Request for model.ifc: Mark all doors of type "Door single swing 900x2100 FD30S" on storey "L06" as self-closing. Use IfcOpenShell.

First a look at what the model holds.

```python
import ifcopenshell
import ifcopenshell.util.element

model = ifcopenshell.open("model.ifc")
print(model.schema)
storey = next(s for s in model.by_type("IfcBuildingStorey") if s.Name == "L06")
doors = [e for e in ifcopenshell.util.element.get_decomposition(storey) if e.is_a("IfcDoor")]
seen = {}
for e in doors:
    element_type = ifcopenshell.util.element.get_type(e)
    key = (element_type.Name if element_type != e and element_type else None, ifcopenshell.util.element.get_pset(e, "Pset_DoorCommon", "SelfClosing"))
    seen[key] = seen.get(key, 0) + 1
for (name, value), count in sorted(seen.items(), key=str):
    print(count, "x", name, "|", value)
```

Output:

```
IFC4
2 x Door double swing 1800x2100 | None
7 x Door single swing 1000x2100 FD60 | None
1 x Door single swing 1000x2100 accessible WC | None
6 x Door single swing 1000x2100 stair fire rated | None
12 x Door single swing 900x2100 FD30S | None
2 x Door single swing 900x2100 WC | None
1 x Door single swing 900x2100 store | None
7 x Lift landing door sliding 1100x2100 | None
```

```python
import ifcopenshell
import ifcopenshell.api.pset
import ifcopenshell.util.element

model = ifcopenshell.open("model.ifc")

storey = next(s for s in model.by_type("IfcBuildingStorey") if s.Name == "L06")
doors = [e for e in ifcopenshell.util.element.get_decomposition(storey) if e.is_a("IfcDoor")]

count = 0
for e in doors:
    element_type = ifcopenshell.util.element.get_type(e)
    if element_type in (None, e) or element_type.Name != "Door single swing 900x2100 FD30S":
        continue
    # add_pset returns the element's existing set when there is one.
    pset = ifcopenshell.api.pset.add_pset(model, product=e, name="Pset_DoorCommon")
    ifcopenshell.api.pset.edit_pset(model, pset=pset, properties={"SelfClosing": True})
    count += 1

print(count, "doors updated")

model.write("model_rev.ifc")
```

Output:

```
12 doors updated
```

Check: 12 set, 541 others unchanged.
